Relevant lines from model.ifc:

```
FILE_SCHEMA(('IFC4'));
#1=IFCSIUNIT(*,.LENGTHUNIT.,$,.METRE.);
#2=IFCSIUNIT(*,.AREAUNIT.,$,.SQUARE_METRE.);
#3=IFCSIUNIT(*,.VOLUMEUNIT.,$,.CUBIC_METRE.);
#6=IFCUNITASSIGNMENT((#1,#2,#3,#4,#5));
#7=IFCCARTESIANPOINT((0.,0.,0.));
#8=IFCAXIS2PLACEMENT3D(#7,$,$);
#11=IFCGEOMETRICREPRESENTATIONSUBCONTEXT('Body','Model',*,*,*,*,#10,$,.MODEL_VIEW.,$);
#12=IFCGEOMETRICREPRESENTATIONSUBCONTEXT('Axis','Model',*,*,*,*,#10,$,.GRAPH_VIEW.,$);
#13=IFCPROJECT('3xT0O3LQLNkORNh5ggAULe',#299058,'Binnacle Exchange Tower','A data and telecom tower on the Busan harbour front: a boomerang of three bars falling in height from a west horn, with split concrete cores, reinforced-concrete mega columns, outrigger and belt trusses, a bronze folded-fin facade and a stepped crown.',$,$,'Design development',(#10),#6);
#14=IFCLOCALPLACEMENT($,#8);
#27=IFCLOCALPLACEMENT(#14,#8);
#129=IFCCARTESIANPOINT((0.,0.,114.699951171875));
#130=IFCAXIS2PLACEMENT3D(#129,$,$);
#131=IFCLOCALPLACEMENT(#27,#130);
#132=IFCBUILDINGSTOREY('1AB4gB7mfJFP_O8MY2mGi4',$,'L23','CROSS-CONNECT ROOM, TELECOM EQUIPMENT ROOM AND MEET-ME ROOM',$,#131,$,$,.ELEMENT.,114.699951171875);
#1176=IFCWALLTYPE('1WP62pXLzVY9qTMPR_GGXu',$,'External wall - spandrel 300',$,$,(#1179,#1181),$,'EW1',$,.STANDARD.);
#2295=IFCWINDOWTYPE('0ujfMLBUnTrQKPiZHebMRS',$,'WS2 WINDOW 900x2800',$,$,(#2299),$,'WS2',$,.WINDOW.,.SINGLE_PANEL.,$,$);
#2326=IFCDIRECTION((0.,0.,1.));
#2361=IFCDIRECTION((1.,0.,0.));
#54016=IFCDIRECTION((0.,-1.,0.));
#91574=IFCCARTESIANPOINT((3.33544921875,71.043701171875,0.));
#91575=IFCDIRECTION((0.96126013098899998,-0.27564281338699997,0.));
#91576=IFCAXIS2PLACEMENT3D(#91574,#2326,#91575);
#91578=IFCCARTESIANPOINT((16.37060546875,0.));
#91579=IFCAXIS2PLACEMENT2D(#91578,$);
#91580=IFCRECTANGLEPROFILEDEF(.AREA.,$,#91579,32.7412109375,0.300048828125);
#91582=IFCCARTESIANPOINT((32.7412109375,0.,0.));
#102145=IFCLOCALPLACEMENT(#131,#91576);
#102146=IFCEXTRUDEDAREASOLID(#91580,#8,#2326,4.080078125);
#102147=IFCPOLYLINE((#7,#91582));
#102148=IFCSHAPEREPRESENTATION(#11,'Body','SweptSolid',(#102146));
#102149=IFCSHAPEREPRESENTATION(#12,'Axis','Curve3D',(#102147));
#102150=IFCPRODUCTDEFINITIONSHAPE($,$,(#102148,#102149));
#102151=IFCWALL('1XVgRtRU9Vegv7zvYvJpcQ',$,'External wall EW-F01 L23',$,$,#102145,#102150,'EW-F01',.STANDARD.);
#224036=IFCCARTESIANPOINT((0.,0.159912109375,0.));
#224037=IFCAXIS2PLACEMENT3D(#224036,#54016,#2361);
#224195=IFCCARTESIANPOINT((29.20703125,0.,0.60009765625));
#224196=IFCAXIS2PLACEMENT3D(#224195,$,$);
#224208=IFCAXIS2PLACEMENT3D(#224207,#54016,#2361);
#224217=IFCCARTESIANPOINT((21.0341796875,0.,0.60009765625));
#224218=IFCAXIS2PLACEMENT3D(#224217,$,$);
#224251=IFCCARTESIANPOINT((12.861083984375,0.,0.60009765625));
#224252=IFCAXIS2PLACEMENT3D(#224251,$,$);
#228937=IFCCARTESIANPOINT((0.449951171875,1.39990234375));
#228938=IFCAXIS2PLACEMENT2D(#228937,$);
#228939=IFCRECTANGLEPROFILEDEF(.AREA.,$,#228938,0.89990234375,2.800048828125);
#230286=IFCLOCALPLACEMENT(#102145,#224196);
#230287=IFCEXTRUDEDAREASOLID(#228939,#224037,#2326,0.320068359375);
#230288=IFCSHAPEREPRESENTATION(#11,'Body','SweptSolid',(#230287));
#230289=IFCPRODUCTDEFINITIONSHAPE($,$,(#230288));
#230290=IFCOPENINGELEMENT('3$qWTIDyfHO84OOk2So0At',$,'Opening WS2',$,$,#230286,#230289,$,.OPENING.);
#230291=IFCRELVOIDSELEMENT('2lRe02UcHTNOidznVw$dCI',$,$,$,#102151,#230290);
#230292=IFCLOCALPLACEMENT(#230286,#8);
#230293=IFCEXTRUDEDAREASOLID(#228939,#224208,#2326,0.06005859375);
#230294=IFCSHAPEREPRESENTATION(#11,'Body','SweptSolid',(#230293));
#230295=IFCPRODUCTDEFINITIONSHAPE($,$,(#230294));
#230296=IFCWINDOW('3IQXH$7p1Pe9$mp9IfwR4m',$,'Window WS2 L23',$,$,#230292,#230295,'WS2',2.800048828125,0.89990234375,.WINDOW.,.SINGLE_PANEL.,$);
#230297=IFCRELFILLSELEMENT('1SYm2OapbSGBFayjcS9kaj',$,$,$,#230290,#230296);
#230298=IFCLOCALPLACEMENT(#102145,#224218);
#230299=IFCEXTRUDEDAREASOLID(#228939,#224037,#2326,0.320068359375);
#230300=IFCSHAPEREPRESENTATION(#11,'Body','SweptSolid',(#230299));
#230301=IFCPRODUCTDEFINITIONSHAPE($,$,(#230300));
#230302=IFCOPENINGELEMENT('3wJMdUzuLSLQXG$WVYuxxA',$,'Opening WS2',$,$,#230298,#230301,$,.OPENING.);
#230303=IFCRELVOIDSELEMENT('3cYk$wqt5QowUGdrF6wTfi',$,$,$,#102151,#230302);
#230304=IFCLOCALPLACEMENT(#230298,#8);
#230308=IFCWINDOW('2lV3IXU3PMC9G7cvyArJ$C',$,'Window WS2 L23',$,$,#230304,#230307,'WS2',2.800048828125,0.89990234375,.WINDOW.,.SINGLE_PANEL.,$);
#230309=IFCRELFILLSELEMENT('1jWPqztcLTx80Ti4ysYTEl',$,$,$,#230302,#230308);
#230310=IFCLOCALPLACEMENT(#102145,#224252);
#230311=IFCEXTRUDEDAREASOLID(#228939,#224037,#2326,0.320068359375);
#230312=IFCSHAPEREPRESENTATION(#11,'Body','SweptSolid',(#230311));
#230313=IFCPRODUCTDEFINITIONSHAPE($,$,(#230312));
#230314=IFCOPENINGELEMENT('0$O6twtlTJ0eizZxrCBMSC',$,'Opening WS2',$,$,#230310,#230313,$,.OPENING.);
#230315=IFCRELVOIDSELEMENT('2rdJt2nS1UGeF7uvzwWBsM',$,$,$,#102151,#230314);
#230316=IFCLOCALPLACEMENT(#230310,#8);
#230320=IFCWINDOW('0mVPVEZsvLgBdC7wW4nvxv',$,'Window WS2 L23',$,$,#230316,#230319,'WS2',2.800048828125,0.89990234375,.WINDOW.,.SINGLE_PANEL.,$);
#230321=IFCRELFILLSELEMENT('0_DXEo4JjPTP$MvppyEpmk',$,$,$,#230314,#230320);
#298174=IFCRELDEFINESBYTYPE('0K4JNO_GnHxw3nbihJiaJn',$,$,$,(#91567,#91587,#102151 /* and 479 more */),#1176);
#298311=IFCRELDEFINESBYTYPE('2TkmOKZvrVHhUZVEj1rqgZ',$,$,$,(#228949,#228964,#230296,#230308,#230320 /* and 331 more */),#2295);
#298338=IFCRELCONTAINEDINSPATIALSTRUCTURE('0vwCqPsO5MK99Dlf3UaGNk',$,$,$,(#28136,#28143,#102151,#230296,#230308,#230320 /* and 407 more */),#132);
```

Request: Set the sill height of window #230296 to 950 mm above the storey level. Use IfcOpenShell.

```python
import numpy as np
import ifcopenshell
import ifcopenshell.api.geometry
import ifcopenshell.geom
import ifcopenshell.util.element
import ifcopenshell.util.placement
import ifcopenshell.util.shape
import ifcopenshell.util.unit

model = ifcopenshell.open("model.ifc")
unit_scale = ifcopenshell.util.unit.calculate_unit_scale(model)

window = model.by_id(230296)
opening = window.FillsVoids[0].RelatingOpeningElement
storey = ifcopenshell.util.element.get_container(window, ifc_class="IfcBuildingStorey")
level = ifcopenshell.util.placement.get_local_placement(storey.ObjectPlacement)[2, 3]

# The opening's origin need not be at the sill, so measure its lowest point.
shape = ifcopenshell.geom.create_shape(ifcopenshell.geom.settings(), opening)
bottom = ifcopenshell.util.shape.get_shape_bottom_elevation(shape, shape.geometry) / unit_scale
dz = level + 0.95 - bottom

shift = np.array([0.0, 0.0, dz])
# The window is placed relative to its opening, so it follows when the opening moves.
matrix = ifcopenshell.util.placement.get_local_placement(opening.ObjectPlacement)
matrix[:3, 3] += shift
ifcopenshell.api.geometry.edit_object_placement(
    model, product=opening, matrix=matrix, is_si=False, should_transform_children=True
)

print(f"moved by {dz * unit_scale:+.3f} m")

model.write("model_edited.ifc")
```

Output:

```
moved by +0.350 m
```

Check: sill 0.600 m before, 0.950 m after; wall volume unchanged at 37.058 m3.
